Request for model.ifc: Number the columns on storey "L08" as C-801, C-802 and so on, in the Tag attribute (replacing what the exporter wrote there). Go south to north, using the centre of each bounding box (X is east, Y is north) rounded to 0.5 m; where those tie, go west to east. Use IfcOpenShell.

First a look at what the model holds.

```python
import ifcopenshell
import ifcopenshell.util.element
import ifcopenshell.util.placement

model = ifcopenshell.open("model.ifc")
print(model.schema)
storey = next(s for s in model.by_type("IfcBuildingStorey") if s.Name == "L08")
columns = [e for e in ifcopenshell.util.element.get_decomposition(storey) if e.is_a("IfcColumn")]
for e in sorted(columns, key=lambda e: e.id()):
    origin = ifcopenshell.util.placement.get_local_placement(e.ObjectPlacement)[:3, 3]
    print(e.id(), e.Tag, e.Name, origin.round(2) + 0.0, sep=" | ")
```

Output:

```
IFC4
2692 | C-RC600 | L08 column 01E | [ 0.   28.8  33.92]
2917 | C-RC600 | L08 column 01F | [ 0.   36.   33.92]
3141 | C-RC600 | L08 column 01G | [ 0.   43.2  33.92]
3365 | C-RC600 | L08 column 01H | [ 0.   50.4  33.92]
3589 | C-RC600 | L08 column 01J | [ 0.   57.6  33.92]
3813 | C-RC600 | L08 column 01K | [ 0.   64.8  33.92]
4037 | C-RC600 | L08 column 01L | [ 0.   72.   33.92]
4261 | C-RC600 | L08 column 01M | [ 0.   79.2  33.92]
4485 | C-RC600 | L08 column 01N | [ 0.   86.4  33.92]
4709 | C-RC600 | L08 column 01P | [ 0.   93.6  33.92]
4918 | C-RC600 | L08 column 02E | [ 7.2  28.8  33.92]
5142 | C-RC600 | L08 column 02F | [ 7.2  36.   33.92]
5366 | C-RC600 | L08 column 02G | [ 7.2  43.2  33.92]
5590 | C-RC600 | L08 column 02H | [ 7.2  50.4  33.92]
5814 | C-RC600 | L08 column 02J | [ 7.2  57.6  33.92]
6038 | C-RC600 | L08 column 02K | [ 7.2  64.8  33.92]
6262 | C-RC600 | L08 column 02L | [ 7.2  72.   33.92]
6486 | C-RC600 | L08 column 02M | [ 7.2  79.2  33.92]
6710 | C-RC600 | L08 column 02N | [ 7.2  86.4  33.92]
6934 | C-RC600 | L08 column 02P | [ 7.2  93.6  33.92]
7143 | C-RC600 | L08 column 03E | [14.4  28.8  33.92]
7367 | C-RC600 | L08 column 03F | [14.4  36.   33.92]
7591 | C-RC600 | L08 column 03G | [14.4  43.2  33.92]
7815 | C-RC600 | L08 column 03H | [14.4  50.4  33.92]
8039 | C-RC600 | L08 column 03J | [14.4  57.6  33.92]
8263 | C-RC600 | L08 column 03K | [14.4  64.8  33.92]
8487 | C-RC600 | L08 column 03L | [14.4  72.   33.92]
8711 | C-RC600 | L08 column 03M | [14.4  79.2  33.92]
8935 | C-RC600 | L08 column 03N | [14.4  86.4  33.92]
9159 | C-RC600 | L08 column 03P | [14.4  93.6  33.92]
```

```python
import ifcopenshell
import ifcopenshell.geom
import ifcopenshell.util.element
import ifcopenshell.util.shape

model = ifcopenshell.open("model.ifc")
settings = ifcopenshell.geom.settings()
settings.set("use-world-coords", True)


def centre(element):
    shape = ifcopenshell.geom.create_shape(settings, element)
    return ifcopenshell.util.shape.get_bbox_centroid(shape.geometry)


storey = next(s for s in model.by_type("IfcBuildingStorey") if s.Name == "L08")
columns = [e for e in ifcopenshell.util.element.get_decomposition(storey) if e.is_a("IfcColumn")]

# Insertion points can sit at a corner or the storey origin, so sort by the geometry (in metres).
centres = {e: centre(e) for e in columns}
columns.sort(key=lambda e: (round(centres[e][1] / 0.5), centres[e][0]))

for i, e in enumerate(columns, start=1):
    number = f"C-8{i:02d}"
    e.Tag = number
    print(e.id(), number)

model.write("model_rev.ifc")
```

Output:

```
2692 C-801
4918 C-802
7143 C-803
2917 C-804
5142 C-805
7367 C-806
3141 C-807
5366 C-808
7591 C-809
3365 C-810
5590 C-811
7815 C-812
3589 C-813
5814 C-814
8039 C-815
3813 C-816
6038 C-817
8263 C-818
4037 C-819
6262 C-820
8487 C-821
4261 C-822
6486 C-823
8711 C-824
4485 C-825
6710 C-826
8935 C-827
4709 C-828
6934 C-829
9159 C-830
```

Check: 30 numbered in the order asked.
